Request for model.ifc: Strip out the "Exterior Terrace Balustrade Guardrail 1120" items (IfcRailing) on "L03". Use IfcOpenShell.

First a look at what the model holds.

```python
import ifcopenshell
import ifcopenshell.util.element

model = ifcopenshell.open("model.ifc")
print(model.schema)
storey = next(s for s in model.by_type("IfcBuildingStorey") if s.Name == "L03")
railings = [e for e in ifcopenshell.util.element.get_decomposition(storey) if e.is_a("IfcRailing")]
seen = {}
for e in railings:
    element_type = ifcopenshell.util.element.get_type(e)
    name = element_type.Name if element_type not in (None, e) else None
    seen[name] = seen.get(name, 0) + 1
for name, count in sorted(seen.items(), key=str):
    print(count, "x", name)
```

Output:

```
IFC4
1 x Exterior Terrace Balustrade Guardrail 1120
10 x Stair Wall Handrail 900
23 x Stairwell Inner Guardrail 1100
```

```python
import ifcopenshell
import ifcopenshell.api.root
import ifcopenshell.util.element

model = ifcopenshell.open("model.ifc")

storey = next(s for s in model.by_type("IfcBuildingStorey") if s.Name == "L03")
railings = [e for e in ifcopenshell.util.element.get_decomposition(storey) if e.is_a("IfcRailing")]
targets = [e for e in railings if (t := ifcopenshell.util.element.get_type(e)) not in (None, e) and t.Name == "Exterior Terrace Balustrade Guardrail 1120"]

for e in targets:
    ifcopenshell.api.root.remove_product(model, product=e)
print(len(targets), "removed")

model.write("model_edited.ifc")
```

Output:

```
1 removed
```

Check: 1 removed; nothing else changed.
